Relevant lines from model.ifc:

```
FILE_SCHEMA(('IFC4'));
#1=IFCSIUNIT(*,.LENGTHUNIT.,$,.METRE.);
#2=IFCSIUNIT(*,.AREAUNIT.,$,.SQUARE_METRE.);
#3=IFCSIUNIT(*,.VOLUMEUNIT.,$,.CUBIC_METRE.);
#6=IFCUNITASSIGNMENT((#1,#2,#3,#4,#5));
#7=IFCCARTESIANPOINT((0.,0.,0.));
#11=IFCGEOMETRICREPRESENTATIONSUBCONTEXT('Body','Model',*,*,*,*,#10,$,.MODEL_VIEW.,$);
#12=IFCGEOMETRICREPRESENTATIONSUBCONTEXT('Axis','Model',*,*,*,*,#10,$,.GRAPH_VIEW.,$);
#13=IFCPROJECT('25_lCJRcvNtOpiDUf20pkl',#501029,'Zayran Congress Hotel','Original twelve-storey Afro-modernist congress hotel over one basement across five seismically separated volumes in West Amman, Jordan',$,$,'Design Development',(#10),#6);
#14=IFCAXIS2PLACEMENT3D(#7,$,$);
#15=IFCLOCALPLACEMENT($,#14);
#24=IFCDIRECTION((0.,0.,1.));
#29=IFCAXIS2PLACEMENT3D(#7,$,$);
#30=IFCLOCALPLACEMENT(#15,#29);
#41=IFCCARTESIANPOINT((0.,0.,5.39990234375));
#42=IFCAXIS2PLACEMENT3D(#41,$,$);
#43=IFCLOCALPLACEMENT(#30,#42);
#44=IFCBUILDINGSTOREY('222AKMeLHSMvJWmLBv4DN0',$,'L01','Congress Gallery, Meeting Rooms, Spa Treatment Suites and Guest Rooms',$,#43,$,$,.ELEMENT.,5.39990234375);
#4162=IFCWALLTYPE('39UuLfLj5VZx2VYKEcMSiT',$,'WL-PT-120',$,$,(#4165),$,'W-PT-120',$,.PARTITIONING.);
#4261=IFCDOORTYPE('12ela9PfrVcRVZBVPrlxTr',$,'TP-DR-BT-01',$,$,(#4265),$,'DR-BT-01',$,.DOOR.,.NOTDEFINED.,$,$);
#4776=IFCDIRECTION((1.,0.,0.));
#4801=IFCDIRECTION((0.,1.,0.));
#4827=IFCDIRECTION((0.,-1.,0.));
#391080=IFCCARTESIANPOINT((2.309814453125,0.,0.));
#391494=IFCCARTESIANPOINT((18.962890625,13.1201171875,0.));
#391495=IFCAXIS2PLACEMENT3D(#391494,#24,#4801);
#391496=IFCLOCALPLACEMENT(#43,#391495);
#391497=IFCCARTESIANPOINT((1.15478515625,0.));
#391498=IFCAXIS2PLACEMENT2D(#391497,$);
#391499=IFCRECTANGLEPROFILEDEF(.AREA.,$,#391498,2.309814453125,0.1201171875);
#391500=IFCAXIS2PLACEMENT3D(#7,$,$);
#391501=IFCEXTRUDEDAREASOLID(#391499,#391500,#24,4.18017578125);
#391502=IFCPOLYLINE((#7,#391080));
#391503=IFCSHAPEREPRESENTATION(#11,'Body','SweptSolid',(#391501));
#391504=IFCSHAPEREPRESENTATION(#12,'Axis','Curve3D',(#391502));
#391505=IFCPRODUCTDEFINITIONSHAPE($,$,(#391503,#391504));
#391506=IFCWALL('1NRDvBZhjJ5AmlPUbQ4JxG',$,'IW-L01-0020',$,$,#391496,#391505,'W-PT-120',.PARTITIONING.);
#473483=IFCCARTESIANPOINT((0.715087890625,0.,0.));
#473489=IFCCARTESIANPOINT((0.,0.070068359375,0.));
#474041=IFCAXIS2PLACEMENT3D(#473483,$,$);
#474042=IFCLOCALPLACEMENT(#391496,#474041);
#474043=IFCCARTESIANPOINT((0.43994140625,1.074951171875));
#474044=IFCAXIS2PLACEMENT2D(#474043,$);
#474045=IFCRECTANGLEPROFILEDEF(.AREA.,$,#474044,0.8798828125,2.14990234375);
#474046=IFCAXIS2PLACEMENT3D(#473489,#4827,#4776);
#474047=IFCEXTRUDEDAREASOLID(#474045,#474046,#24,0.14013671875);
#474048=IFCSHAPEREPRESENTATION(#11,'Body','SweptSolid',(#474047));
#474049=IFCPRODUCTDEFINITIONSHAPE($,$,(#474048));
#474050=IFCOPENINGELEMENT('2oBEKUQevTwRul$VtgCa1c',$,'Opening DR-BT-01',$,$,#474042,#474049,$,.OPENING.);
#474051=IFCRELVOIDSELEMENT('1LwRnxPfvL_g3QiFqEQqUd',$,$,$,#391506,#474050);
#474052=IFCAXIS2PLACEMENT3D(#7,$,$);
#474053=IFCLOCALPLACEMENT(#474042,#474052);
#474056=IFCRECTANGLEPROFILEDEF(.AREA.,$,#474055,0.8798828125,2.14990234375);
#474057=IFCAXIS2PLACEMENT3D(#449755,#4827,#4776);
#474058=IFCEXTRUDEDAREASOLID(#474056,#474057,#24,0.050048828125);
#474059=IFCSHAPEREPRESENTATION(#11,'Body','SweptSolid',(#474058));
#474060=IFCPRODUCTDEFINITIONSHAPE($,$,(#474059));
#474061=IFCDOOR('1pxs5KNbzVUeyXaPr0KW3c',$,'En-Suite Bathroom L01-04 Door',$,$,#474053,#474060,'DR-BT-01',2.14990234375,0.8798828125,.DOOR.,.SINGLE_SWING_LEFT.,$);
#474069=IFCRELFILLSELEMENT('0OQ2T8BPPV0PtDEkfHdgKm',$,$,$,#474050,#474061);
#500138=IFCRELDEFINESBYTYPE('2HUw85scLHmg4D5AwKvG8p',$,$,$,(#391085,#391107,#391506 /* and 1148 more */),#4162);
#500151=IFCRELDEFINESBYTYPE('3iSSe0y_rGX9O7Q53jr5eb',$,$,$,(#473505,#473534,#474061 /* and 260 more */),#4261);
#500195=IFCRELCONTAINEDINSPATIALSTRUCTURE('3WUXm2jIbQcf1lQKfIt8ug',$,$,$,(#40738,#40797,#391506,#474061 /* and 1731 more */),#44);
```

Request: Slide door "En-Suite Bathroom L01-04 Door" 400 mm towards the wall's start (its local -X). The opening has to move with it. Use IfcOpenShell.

```python
import ifcopenshell
import ifcopenshell.api.geometry
import ifcopenshell.util.placement
import ifcopenshell.util.unit

model = ifcopenshell.open("model.ifc")
unit_scale = ifcopenshell.util.unit.calculate_unit_scale(model)

door = model.by_guid("1pxs5KNbzVUeyXaPr0KW3c")
opening = door.FillsVoids[0].RelatingOpeningElement
wall = opening.VoidsElements[0].RelatingBuildingElement

wall_matrix = ifcopenshell.util.placement.get_local_placement(wall.ObjectPlacement)
shift = wall_matrix[:3, 0] * -0.4 / unit_scale
before = ifcopenshell.util.placement.get_local_placement(door.ObjectPlacement)[:3, 3].copy()

# The door is placed relative to its opening, so it follows when the opening moves.
matrix = ifcopenshell.util.placement.get_local_placement(opening.ObjectPlacement)
matrix[:3, 3] += shift
ifcopenshell.api.geometry.edit_object_placement(
    model, product=opening, matrix=matrix, is_si=False, should_transform_children=True
)

after = ifcopenshell.util.placement.get_local_placement(door.ObjectPlacement)[:3, 3]
print("door moved by", (after - before).round(3) + 0.0)

model.write("model_updated.ifc")
```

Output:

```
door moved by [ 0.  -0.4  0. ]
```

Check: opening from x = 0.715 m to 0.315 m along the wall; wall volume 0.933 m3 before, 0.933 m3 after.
